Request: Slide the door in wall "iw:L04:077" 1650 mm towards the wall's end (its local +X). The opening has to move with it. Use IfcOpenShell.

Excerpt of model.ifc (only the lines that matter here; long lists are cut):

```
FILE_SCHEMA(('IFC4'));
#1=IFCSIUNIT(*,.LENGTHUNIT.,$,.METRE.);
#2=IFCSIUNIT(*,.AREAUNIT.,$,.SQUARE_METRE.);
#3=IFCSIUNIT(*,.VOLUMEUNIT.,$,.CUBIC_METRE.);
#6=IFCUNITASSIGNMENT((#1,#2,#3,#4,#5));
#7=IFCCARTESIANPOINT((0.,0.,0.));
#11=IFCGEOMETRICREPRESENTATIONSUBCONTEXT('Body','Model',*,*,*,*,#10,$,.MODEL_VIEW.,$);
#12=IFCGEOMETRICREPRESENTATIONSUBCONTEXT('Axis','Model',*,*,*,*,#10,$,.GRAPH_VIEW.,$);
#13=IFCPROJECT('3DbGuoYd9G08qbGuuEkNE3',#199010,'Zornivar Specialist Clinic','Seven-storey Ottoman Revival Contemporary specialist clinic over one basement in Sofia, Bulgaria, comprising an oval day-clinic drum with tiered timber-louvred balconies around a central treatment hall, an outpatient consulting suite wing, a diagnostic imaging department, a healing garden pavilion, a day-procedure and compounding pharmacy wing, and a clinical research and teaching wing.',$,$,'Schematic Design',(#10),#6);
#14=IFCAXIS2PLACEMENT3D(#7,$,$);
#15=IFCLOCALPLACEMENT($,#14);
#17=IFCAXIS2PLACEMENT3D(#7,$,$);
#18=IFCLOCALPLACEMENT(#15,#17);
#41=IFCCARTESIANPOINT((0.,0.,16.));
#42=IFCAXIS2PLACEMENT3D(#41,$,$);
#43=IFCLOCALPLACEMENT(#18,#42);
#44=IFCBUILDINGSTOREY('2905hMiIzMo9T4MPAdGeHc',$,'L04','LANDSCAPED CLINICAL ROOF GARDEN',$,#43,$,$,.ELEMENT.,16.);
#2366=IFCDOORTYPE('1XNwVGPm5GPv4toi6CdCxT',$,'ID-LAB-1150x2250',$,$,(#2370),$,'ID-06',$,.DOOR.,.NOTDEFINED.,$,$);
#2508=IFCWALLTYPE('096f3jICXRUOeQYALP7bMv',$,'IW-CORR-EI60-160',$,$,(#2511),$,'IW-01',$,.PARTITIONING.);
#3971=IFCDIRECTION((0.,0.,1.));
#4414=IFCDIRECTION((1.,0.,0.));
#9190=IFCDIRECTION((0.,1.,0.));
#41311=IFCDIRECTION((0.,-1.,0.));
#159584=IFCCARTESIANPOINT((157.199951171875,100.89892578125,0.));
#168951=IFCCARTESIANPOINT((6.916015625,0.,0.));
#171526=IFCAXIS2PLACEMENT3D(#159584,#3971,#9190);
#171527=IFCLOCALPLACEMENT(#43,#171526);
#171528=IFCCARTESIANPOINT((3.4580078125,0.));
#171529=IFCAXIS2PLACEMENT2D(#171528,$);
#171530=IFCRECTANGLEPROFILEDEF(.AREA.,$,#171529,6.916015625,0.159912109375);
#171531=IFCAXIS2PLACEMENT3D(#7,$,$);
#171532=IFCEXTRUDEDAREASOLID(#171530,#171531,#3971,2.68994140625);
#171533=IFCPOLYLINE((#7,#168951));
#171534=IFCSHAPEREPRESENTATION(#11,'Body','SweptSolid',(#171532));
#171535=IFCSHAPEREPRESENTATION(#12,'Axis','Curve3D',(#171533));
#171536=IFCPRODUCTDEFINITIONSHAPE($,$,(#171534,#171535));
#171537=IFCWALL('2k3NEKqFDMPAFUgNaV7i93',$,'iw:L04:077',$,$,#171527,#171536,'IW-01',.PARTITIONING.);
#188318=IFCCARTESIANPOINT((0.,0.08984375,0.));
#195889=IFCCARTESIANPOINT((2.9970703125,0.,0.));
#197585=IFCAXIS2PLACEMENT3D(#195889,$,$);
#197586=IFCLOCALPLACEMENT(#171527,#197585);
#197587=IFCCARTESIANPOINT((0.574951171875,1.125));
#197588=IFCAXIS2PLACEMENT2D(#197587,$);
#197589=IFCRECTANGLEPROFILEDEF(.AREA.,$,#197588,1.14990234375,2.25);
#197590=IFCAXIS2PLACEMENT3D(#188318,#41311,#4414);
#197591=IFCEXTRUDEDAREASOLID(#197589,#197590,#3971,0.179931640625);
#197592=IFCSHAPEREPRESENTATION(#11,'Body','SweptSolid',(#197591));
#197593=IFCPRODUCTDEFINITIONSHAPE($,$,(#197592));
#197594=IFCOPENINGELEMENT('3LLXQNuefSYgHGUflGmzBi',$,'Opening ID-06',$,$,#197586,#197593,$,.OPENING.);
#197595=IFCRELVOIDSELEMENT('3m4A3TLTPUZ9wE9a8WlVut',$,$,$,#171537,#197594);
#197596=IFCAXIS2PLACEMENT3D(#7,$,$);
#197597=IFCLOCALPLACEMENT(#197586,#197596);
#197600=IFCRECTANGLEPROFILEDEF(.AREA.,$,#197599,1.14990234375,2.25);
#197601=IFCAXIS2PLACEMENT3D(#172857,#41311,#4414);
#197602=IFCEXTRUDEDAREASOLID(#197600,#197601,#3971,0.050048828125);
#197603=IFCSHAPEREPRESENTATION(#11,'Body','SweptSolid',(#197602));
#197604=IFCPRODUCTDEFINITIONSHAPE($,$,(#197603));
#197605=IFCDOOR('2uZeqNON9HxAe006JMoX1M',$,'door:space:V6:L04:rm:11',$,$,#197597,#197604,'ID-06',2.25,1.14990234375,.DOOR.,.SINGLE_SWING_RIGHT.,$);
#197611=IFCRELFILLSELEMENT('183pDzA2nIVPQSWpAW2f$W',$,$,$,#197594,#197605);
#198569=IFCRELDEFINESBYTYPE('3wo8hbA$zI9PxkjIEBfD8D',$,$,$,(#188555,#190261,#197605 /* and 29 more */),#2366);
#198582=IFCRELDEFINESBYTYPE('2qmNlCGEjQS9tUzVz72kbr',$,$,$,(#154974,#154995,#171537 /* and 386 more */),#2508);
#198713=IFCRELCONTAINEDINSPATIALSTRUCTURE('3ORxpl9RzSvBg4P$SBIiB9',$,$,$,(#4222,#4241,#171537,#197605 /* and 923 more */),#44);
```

```python
import ifcopenshell
import ifcopenshell.api.geometry
import ifcopenshell.util.placement

model = ifcopenshell.open("model.ifc")

door = model.by_id(197605)
opening = door.FillsVoids[0].RelatingOpeningElement
wall = opening.VoidsElements[0].RelatingBuildingElement

wall_matrix = ifcopenshell.util.placement.get_local_placement(wall.ObjectPlacement)
shift = wall_matrix[:3, 0] * 1.65
before = ifcopenshell.util.placement.get_local_placement(door.ObjectPlacement)[:3, 3].copy()

# The door is placed relative to its opening, so it follows when the opening moves.
matrix = ifcopenshell.util.placement.get_local_placement(opening.ObjectPlacement)
matrix[:3, 3] += shift
ifcopenshell.api.geometry.edit_object_placement(
    model, product=opening, matrix=matrix, is_si=False, should_transform_children=True
)

after = ifcopenshell.util.placement.get_local_placement(door.ObjectPlacement)[:3, 3]
print("door moved by", (after - before).round(3) + 0.0)

model.write("model_updated.ifc")
```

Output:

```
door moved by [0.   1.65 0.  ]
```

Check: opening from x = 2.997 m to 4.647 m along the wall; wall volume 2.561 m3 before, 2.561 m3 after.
